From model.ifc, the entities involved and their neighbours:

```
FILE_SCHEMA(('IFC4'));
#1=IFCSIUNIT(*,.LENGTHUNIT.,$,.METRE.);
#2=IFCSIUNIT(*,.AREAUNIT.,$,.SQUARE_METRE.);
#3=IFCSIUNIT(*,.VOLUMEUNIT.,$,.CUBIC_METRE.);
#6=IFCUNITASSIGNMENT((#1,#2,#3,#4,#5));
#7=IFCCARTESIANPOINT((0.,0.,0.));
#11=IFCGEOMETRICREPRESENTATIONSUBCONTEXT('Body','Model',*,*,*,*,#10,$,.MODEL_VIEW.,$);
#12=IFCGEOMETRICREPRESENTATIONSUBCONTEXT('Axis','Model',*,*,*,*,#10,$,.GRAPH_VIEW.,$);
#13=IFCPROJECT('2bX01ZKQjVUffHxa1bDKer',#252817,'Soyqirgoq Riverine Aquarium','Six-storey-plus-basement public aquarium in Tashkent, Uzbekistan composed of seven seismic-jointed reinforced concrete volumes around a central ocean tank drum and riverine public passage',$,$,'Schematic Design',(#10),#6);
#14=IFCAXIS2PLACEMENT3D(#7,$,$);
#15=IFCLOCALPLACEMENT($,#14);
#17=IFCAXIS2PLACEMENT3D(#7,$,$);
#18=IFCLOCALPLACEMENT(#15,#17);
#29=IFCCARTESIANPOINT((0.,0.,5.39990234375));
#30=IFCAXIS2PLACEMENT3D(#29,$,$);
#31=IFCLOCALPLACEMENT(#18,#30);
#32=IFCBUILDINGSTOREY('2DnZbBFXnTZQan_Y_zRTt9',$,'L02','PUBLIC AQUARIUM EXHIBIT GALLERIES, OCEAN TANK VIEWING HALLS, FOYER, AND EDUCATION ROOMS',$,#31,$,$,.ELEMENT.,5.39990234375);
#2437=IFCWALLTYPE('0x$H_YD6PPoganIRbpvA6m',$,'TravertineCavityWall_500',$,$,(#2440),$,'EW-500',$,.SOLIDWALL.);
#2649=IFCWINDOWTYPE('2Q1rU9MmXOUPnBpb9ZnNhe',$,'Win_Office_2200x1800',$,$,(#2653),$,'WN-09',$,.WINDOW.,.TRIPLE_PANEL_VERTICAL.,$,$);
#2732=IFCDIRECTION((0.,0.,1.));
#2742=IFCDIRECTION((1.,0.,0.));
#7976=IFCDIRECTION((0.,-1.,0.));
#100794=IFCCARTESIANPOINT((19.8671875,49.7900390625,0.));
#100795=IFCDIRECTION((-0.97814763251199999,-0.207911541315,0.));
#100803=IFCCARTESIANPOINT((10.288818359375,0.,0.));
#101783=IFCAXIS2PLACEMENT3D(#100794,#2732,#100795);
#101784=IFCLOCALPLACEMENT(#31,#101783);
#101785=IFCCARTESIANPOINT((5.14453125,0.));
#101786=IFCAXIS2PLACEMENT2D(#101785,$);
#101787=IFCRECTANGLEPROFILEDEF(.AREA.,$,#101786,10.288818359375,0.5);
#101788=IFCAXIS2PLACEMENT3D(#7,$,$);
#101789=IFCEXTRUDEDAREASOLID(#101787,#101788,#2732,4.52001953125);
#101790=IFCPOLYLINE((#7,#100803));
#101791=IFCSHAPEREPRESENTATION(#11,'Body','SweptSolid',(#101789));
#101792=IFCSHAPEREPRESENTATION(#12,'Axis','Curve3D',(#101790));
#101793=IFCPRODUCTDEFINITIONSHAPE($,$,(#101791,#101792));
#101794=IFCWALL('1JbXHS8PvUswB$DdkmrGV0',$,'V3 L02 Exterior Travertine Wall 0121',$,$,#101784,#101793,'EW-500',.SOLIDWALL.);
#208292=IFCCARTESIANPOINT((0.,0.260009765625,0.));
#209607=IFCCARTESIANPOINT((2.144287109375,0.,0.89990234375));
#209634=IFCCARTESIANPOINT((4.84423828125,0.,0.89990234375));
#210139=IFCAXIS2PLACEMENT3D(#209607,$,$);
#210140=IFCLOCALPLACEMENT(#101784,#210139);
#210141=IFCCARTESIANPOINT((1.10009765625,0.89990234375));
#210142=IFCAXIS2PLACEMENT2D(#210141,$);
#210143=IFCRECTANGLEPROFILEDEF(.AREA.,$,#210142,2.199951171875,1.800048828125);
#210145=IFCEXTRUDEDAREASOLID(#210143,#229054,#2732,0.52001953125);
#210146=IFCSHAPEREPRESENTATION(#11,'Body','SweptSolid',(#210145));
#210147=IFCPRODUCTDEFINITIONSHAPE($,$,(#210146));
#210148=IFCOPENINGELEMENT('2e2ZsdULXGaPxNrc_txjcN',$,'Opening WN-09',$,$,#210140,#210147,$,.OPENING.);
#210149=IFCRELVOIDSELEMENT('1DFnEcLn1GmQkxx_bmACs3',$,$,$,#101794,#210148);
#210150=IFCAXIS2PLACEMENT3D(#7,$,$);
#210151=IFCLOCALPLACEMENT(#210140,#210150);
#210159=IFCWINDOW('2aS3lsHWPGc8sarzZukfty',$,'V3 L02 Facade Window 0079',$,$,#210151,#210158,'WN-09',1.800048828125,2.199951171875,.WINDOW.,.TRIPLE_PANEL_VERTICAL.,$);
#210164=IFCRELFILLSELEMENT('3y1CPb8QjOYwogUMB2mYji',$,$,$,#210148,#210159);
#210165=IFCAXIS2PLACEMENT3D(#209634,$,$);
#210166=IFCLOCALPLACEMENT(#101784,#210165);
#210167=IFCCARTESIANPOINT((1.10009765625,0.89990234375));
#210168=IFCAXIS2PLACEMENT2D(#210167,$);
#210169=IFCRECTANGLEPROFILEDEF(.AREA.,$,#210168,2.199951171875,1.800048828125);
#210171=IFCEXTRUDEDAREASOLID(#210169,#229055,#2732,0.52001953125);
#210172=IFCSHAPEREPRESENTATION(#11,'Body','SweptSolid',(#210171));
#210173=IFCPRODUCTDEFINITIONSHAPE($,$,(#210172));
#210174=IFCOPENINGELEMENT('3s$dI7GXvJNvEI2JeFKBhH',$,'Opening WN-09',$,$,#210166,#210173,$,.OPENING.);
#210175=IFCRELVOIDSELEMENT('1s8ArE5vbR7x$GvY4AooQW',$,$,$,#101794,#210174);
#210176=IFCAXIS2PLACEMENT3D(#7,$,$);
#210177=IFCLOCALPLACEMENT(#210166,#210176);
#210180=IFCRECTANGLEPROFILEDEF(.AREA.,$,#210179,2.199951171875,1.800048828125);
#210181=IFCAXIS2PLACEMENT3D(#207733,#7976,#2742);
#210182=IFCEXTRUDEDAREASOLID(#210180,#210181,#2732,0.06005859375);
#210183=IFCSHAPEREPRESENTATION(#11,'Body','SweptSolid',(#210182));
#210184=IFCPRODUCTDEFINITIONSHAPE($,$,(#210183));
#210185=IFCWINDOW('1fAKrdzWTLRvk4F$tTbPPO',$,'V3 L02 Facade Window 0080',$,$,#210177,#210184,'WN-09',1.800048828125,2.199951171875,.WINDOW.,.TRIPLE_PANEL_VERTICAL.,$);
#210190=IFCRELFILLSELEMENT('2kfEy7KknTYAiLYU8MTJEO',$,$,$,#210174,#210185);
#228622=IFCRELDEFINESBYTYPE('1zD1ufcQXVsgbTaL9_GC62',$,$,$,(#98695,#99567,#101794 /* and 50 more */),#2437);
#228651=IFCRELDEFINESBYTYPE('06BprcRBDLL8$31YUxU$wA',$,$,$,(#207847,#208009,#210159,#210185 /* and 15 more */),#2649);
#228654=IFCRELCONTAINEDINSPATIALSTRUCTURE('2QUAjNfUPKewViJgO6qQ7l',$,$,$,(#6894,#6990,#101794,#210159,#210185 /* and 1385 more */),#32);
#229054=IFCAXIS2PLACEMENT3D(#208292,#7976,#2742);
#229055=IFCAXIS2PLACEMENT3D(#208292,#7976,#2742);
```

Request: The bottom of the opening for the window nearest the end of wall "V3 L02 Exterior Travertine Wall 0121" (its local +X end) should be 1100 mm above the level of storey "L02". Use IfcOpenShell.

```python
import numpy as np
import ifcopenshell
import ifcopenshell.api.geometry
import ifcopenshell.geom
import ifcopenshell.util.element
import ifcopenshell.util.placement
import ifcopenshell.util.shape
import ifcopenshell.util.unit

model = ifcopenshell.open("model.ifc")
unit_scale = ifcopenshell.util.unit.calculate_unit_scale(model)

window = model.by_guid("1fAKrdzWTLRvk4F$tTbPPO")
opening = window.FillsVoids[0].RelatingOpeningElement
storey = ifcopenshell.util.element.get_container(window, ifc_class="IfcBuildingStorey")
level = ifcopenshell.util.placement.get_local_placement(storey.ObjectPlacement)[2, 3]

# The opening's origin need not be at the sill, so measure its lowest point.
shape = ifcopenshell.geom.create_shape(ifcopenshell.geom.settings(), opening)
bottom = ifcopenshell.util.shape.get_shape_bottom_elevation(shape, shape.geometry) / unit_scale
dz = level + 1.1 / unit_scale - bottom

shift = np.array([0.0, 0.0, dz])
# The window is placed relative to its opening, so it follows when the opening moves.
matrix = ifcopenshell.util.placement.get_local_placement(opening.ObjectPlacement)
matrix[:3, 3] += shift
ifcopenshell.api.geometry.edit_object_placement(
    model, product=opening, matrix=matrix, is_si=False, should_transform_children=True
)

print(f"moved by {dz * unit_scale:+.3f} m")

model.write("model_v2.ifc")
```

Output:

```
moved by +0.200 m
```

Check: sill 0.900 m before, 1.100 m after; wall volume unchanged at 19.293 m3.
